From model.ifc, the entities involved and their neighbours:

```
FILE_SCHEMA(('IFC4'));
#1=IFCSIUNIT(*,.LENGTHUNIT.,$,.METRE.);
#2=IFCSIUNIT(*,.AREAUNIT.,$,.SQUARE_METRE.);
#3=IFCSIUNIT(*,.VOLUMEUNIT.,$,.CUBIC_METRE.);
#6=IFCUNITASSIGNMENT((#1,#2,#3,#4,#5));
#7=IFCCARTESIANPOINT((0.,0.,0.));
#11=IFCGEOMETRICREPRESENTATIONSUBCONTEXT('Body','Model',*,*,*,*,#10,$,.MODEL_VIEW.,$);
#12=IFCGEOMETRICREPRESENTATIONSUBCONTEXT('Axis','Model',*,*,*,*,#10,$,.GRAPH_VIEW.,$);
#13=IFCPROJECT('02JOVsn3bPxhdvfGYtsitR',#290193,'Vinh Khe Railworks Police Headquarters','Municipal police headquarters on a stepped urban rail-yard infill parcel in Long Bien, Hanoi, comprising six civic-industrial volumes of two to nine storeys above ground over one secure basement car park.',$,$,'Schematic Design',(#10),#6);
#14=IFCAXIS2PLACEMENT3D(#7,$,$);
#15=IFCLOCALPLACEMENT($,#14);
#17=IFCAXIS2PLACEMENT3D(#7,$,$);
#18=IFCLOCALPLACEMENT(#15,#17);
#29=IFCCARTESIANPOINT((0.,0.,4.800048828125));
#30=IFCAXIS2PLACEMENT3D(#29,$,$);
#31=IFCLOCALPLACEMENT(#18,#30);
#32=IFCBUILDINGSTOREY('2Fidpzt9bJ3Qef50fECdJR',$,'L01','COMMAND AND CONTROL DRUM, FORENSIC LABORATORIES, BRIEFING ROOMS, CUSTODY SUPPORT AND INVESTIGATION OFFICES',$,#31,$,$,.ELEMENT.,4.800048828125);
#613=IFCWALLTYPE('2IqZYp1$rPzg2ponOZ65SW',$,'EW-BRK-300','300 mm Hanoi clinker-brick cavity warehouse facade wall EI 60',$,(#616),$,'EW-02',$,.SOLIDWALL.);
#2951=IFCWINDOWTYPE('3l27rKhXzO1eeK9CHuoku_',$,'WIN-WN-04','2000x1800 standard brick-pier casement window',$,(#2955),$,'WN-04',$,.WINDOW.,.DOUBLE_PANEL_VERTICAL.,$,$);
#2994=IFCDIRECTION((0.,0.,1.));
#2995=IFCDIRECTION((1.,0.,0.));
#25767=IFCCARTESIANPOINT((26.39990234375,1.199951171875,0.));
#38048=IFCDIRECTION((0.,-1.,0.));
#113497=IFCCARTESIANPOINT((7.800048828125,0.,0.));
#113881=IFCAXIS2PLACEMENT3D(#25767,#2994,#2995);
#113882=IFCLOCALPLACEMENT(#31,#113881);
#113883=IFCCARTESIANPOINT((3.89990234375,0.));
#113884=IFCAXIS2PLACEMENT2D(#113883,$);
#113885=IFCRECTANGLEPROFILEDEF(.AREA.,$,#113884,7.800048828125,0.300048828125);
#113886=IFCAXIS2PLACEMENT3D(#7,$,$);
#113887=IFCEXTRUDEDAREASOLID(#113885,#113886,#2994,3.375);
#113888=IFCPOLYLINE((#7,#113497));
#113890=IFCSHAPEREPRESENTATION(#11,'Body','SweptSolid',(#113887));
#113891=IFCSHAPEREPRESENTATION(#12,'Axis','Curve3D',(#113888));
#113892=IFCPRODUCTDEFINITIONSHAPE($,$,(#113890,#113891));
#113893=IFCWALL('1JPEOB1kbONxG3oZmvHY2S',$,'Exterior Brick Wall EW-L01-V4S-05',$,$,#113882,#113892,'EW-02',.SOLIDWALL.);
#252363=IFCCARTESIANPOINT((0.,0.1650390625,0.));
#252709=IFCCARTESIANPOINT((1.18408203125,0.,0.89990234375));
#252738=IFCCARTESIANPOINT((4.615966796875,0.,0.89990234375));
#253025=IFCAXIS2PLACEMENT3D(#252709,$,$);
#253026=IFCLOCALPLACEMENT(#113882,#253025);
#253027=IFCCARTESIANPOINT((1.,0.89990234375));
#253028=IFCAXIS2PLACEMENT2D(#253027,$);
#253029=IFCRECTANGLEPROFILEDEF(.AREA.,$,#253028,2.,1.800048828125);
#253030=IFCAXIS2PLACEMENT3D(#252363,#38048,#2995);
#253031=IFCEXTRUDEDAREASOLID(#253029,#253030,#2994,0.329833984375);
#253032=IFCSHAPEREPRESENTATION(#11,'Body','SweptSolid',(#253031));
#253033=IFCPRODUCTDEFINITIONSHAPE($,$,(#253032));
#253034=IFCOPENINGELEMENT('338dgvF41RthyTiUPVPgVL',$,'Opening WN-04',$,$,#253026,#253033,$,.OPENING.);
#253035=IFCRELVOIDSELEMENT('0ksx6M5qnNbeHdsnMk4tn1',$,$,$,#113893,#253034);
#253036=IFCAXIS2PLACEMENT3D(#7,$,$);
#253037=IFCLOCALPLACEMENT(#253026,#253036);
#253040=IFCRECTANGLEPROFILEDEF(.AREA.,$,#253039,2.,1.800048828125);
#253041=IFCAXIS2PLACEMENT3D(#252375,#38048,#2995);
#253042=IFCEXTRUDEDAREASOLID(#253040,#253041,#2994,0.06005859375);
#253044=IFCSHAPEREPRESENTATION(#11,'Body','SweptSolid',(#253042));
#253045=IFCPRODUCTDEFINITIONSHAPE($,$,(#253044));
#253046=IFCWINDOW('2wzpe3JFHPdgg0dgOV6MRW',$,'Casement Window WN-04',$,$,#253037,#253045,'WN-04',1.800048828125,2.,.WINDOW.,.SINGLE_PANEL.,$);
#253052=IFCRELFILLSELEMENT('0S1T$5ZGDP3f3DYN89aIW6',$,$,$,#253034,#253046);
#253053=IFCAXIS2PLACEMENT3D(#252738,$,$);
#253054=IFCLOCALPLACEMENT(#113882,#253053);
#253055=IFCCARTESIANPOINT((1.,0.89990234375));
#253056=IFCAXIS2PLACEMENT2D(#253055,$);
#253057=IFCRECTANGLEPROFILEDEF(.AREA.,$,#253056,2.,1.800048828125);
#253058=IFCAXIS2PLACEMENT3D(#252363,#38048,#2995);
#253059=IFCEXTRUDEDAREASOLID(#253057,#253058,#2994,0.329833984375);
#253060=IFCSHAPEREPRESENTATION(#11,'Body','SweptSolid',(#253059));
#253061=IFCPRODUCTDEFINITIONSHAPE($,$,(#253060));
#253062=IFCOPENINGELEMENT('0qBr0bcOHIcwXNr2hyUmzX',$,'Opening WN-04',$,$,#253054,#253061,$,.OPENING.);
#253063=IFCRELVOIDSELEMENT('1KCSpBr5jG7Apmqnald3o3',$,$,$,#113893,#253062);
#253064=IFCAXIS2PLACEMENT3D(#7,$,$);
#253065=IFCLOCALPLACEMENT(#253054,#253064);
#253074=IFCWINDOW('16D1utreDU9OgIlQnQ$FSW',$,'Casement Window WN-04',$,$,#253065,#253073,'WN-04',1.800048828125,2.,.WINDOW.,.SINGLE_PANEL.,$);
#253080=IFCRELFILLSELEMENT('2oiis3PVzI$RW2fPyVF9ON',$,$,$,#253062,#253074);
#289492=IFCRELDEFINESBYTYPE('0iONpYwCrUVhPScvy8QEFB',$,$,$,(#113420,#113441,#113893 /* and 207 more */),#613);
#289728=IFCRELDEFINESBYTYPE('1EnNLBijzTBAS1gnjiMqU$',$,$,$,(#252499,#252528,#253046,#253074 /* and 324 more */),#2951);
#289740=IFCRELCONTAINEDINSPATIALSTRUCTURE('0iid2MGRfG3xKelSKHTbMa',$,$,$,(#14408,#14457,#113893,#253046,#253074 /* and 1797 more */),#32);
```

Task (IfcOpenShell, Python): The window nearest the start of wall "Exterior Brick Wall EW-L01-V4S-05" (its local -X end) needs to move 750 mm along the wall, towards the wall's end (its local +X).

```python
import ifcopenshell
import ifcopenshell.api.geometry
import ifcopenshell.util.placement

model = ifcopenshell.open("model.ifc")

window = model.by_guid("2wzpe3JFHPdgg0dgOV6MRW")
opening = window.FillsVoids[0].RelatingOpeningElement
wall = opening.VoidsElements[0].RelatingBuildingElement

wall_matrix = ifcopenshell.util.placement.get_local_placement(wall.ObjectPlacement)
shift = wall_matrix[:3, 0] * 0.75
before = ifcopenshell.util.placement.get_local_placement(window.ObjectPlacement)[:3, 3].copy()

# The window is placed relative to its opening, so it follows when the opening moves.
matrix = ifcopenshell.util.placement.get_local_placement(opening.ObjectPlacement)
matrix[:3, 3] += shift
ifcopenshell.api.geometry.edit_object_placement(
    model, product=opening, matrix=matrix, is_si=False, should_transform_children=True
)

after = ifcopenshell.util.placement.get_local_placement(window.ObjectPlacement)[:3, 3]
print("window moved by", (after - before).round(3) + 0.0)

model.write("model_edited.ifc")
```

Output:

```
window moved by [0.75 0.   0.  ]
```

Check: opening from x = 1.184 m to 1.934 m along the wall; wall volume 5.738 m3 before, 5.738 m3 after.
